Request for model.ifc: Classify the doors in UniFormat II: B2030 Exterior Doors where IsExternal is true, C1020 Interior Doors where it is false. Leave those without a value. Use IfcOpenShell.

First a look at what the model holds.

```python
import ifcopenshell
import ifcopenshell.util.element

model = ifcopenshell.open("model.ifc")
print(model.schema)
print("classifications:", [c.Name for c in model.by_type("IfcClassification")])
values = [ifcopenshell.util.element.get_pset(e, "Pset_DoorCommon", "IsExternal") for e in model.by_type("IfcDoor")]
for value in (True, False, None):
    print("IsExternal", value, values.count(value))
```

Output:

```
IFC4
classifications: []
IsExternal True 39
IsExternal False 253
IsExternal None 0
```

```python
import ifcopenshell
import ifcopenshell.api.classification
import ifcopenshell.util.element

model = ifcopenshell.open("model.ifc")

system = ifcopenshell.api.classification.add_classification(model, classification="UniFormat II")

doors = model.by_type("IfcDoor")
external = {e: ifcopenshell.util.element.get_pset(e, "Pset_DoorCommon", "IsExternal") for e in doors}
for flag, code, name in ((True, "B2030", "Exterior Doors"), (False, "C1020", "Interior Doors")):
    products = [e for e in doors if external[e] is flag]
    ifcopenshell.api.classification.add_reference(
        model, products=products, classification=system, identification=code, name=name
    )
    print(code, len(products))

model.write("model_updated.ifc")
```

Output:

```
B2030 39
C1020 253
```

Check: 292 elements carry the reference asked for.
